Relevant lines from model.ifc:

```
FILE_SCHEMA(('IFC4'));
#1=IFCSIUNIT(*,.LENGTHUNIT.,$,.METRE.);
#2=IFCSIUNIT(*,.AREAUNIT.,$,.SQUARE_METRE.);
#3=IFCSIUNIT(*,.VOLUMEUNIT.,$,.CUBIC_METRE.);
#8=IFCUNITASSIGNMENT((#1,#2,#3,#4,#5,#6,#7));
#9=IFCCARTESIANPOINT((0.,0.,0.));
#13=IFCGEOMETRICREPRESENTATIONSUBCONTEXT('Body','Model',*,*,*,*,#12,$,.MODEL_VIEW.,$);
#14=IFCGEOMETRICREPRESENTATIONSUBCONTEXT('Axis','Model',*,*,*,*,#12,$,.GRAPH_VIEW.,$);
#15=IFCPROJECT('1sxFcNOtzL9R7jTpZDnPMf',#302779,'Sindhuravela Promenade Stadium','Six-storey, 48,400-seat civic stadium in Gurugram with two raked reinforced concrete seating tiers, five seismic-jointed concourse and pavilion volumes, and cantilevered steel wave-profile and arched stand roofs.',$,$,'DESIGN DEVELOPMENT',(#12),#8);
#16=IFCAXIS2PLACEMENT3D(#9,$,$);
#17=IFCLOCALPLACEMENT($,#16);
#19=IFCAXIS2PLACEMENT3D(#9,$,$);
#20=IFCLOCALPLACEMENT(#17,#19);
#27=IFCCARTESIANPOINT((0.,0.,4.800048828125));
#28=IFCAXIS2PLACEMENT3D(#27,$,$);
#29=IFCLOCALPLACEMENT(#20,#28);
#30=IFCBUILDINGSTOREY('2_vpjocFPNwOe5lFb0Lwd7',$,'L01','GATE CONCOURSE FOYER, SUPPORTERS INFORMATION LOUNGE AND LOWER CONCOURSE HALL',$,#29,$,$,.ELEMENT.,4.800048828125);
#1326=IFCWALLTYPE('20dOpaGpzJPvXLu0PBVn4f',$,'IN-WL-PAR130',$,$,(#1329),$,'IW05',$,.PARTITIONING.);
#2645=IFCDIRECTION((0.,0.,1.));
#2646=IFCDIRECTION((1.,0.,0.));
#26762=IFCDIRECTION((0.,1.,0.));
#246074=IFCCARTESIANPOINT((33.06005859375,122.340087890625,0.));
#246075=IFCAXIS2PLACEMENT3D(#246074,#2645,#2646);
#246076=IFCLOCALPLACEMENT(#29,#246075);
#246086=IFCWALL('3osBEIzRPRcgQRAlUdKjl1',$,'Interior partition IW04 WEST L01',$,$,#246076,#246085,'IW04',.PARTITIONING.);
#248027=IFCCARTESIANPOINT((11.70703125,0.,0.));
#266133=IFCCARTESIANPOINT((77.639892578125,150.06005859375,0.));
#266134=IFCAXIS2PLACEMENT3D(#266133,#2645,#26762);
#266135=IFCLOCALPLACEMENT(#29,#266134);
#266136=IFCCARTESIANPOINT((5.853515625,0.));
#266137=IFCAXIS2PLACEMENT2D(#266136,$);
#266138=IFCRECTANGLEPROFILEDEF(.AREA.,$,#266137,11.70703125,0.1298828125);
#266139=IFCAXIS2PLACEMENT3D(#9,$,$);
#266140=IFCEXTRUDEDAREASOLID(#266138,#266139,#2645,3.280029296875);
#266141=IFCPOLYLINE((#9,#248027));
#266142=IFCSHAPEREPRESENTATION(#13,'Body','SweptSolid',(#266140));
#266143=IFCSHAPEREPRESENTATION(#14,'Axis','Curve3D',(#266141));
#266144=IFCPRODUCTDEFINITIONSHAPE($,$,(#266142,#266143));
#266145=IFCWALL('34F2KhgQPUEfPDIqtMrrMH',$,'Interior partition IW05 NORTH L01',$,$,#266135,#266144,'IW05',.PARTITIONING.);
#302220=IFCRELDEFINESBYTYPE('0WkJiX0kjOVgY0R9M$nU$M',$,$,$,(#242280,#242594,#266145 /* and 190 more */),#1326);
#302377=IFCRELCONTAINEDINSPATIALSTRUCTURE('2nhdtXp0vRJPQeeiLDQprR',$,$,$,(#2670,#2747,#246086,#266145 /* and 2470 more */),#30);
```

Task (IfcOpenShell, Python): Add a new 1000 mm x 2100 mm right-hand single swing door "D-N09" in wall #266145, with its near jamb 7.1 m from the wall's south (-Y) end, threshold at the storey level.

```python
import numpy as np
import ifcopenshell
import ifcopenshell.api.feature
import ifcopenshell.api.geometry
import ifcopenshell.api.root
import ifcopenshell.api.spatial
import ifcopenshell.geom
import ifcopenshell.util.element
import ifcopenshell.util.placement
import ifcopenshell.util.representation
import ifcopenshell.util.shape
import ifcopenshell.util.unit

model = ifcopenshell.open("model.ifc")
unit_scale = ifcopenshell.util.unit.calculate_unit_scale(model)
settings = ifcopenshell.geom.settings()


def volume(element):
    """Net volume in cubic metres, openings subtracted."""
    shape = ifcopenshell.geom.create_shape(settings, element)
    return ifcopenshell.util.shape.get_volume(shape.geometry)


wall = model.by_guid("34F2KhgQPUEfPDIqtMrrMH")
storey = ifcopenshell.util.element.get_container(wall, ifc_class="IfcBuildingStorey")
context = ifcopenshell.util.representation.get_context(model, "Model", "Body", "MODEL_VIEW")
before = volume(wall)

width, height, from_end, sill = 1, 2.1, 7.1, 0.0  # metres

# The wall runs along its own X axis, and the end named is its -X end.
wall_shape = ifcopenshell.geom.create_shape(settings, wall)
x, y, z = ifcopenshell.util.shape.get_vertices(wall_shape.geometry).T
start = x.min() + from_end
face, thickness = float(y.min()), float(y.max() - y.min())
wall_matrix = ifcopenshell.util.placement.get_local_placement(wall.ObjectPlacement)
level = ifcopenshell.util.placement.get_local_placement(storey.ObjectPlacement)[2, 3]


def in_wall(x, y):
    """Placement at x, y metres in the wall's axes, at sill height."""
    matrix = wall_matrix.copy()
    matrix[:, 3] = wall_matrix @ np.array([x / unit_scale, y / unit_scale, 0.0, 1.0])
    matrix[2, 3] = level + sill / unit_scale
    return matrix


# Opening: a box that overshoots both wall faces by 50 mm.
opening = ifcopenshell.api.root.create_entity(model, ifc_class="IfcOpeningElement", predefined_type="OPENING")
box = ifcopenshell.api.geometry.add_wall_representation(
    model, context=context, length=width, height=height, thickness=thickness + 0.1
)
ifcopenshell.api.geometry.assign_representation(model, product=opening, representation=box)
ifcopenshell.api.geometry.edit_object_placement(model, product=opening, matrix=in_wall(start, face - 0.05), is_si=False)
ifcopenshell.api.feature.add_feature(model, feature=opening, element=wall)

door = ifcopenshell.api.root.create_entity(model, ifc_class="IfcDoor", name="D-N09", predefined_type="DOOR")
door.OverallWidth, door.OverallHeight = width / unit_scale, height / unit_scale
door.OperationType = "SINGLE_SWING_RIGHT"
body = ifcopenshell.api.geometry.add_door_representation(
    model,
    context=context,
    overall_width=door.OverallWidth,
    overall_height=door.OverallHeight,
    operation_type="SINGLE_SWING_RIGHT",
    lining_properties={"LiningDepth": thickness / unit_scale, "ThresholdDepth": thickness / unit_scale},
)
ifcopenshell.api.geometry.assign_representation(model, product=door, representation=body)
ifcopenshell.api.spatial.assign_container(model, products=[door], relating_structure=storey)
ifcopenshell.api.feature.add_filling(model, opening=opening, element=door)

# The lining spans the wall, so the door starts at the wall face.
ifcopenshell.api.geometry.edit_object_placement(model, product=door, matrix=in_wall(start, face), is_si=False)

after = volume(wall)

print(f"wall volume {before:.3f} -> {after:.3f} m3")

model.write("model_edited.ifc")
```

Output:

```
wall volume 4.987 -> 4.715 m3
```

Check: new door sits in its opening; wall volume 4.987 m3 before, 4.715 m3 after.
